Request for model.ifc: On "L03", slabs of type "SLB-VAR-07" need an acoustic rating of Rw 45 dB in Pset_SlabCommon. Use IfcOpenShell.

First a look at what the model holds.

```python
import ifcopenshell
import ifcopenshell.util.element

model = ifcopenshell.open("model.ifc")
print(model.schema)
storey = next(s for s in model.by_type("IfcBuildingStorey") if s.Name == "L03")
slabs = [e for e in ifcopenshell.util.element.get_decomposition(storey) if e.is_a("IfcSlab")]
seen = {}
for e in slabs:
    element_type = ifcopenshell.util.element.get_type(e)
    key = (element_type.Name if element_type != e and element_type else None, ifcopenshell.util.element.get_pset(e, "Pset_SlabCommon", "AcousticRating"))
    seen[key] = seen.get(key, 0) + 1
for (name, value), count in sorted(seen.items(), key=str):
    print(count, "x", name, "|", value)
```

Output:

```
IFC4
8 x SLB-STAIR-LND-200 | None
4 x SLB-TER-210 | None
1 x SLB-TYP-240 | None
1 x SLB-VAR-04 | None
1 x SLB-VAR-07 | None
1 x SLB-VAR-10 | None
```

```python
import ifcopenshell
import ifcopenshell.api.pset
import ifcopenshell.util.element

model = ifcopenshell.open("model.ifc")

storey = next(s for s in model.by_type("IfcBuildingStorey") if s.Name == "L03")
slabs = [e for e in ifcopenshell.util.element.get_decomposition(storey) if e.is_a("IfcSlab")]

count = 0
for e in slabs:
    element_type = ifcopenshell.util.element.get_type(e)
    if element_type in (None, e) or element_type.Name != "SLB-VAR-07":
        continue
    # add_pset returns the element's existing set when there is one.
    pset = ifcopenshell.api.pset.add_pset(model, product=e, name="Pset_SlabCommon")
    ifcopenshell.api.pset.edit_pset(model, pset=pset, properties={"AcousticRating": "Rw 45 dB"})
    count += 1

print(count, "slabs updated")

model.write("model-out.ifc")
```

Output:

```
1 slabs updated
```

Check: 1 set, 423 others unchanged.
